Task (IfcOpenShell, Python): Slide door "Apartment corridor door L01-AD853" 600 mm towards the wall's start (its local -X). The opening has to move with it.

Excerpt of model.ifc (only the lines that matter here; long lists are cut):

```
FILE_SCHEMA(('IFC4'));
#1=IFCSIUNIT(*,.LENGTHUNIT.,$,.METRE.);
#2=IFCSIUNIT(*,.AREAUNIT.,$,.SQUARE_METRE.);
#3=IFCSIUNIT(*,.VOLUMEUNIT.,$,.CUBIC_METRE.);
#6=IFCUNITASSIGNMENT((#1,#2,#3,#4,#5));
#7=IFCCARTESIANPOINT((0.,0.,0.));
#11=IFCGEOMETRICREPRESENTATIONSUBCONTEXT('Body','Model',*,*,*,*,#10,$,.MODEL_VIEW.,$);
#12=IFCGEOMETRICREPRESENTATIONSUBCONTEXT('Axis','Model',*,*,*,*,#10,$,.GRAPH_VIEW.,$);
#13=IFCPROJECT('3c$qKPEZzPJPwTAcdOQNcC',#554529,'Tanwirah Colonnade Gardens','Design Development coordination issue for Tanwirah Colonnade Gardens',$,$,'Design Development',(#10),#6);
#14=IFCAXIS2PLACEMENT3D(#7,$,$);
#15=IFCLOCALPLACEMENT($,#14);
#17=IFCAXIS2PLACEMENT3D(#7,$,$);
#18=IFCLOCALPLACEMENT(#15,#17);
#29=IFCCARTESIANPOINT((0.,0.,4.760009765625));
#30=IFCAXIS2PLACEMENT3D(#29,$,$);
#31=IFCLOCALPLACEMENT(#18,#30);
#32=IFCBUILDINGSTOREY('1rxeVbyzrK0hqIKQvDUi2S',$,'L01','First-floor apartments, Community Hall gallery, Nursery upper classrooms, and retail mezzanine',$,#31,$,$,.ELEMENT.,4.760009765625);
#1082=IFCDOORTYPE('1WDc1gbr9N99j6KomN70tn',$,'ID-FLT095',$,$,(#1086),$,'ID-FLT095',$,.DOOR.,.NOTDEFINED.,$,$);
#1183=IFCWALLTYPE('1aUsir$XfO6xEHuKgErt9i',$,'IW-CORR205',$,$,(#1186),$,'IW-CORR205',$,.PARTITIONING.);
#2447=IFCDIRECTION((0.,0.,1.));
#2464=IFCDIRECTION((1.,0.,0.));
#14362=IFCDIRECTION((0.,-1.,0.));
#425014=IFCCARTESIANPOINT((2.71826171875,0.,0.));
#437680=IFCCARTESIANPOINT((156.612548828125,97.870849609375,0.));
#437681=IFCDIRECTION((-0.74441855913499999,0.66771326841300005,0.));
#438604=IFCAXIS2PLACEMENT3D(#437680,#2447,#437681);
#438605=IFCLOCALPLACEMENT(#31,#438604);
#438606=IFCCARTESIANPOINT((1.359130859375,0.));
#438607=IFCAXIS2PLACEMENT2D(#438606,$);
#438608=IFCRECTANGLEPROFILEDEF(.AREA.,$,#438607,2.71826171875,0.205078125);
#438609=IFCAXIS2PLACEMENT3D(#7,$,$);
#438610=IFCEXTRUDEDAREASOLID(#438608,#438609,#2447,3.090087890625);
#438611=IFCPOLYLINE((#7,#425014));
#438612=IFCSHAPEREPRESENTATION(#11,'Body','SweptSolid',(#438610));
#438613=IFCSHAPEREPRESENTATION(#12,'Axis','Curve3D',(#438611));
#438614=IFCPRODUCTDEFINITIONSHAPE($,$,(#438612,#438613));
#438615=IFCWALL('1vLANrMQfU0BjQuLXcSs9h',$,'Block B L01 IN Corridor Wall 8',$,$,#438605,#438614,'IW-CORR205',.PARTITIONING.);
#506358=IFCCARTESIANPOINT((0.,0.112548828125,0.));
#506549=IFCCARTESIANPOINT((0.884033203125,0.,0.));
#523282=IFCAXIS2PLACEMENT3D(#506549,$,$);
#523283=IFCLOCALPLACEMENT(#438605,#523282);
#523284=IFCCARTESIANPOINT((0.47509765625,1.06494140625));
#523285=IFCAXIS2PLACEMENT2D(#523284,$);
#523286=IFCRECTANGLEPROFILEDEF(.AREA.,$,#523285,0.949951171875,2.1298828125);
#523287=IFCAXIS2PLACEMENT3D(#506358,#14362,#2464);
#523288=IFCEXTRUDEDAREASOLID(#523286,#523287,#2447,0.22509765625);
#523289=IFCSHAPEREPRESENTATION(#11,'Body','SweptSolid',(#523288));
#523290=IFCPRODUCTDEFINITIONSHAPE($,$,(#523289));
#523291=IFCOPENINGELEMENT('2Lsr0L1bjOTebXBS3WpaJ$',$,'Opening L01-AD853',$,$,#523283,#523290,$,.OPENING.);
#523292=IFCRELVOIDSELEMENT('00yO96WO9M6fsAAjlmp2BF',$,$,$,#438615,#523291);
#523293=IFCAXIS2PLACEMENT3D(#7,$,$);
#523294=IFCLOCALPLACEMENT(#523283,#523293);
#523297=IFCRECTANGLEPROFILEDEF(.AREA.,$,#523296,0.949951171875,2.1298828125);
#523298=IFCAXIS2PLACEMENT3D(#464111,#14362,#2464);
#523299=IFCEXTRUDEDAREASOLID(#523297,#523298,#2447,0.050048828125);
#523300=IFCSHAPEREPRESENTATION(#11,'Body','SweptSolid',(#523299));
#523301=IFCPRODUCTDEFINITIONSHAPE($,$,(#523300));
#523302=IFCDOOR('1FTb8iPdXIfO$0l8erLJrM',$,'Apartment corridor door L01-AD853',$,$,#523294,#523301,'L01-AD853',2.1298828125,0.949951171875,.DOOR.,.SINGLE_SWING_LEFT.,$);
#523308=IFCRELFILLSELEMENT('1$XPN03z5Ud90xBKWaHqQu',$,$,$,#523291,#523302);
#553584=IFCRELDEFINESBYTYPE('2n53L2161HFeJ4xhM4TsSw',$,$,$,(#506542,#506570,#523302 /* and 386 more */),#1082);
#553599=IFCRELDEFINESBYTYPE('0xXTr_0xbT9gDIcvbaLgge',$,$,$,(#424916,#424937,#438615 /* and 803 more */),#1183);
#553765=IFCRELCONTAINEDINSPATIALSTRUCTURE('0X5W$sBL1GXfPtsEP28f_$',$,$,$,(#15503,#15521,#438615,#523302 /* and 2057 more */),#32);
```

```python
import ifcopenshell
import ifcopenshell.api.geometry
import ifcopenshell.util.placement

model = ifcopenshell.open("model.ifc")

door = model.by_id(523302)
opening = door.FillsVoids[0].RelatingOpeningElement
wall = opening.VoidsElements[0].RelatingBuildingElement

wall_matrix = ifcopenshell.util.placement.get_local_placement(wall.ObjectPlacement)
shift = wall_matrix[:3, 0] * -0.6
before = ifcopenshell.util.placement.get_local_placement(door.ObjectPlacement)[:3, 3].copy()

# The door is placed relative to its opening, so it follows when the opening moves.
matrix = ifcopenshell.util.placement.get_local_placement(opening.ObjectPlacement)
matrix[:3, 3] += shift
ifcopenshell.api.geometry.edit_object_placement(
    model, product=opening, matrix=matrix, is_si=False, should_transform_children=True
)

after = ifcopenshell.util.placement.get_local_placement(door.ObjectPlacement)[:3, 3]
print("door moved by", (after - before).round(3) + 0.0)

model.write("model_updated.ifc")
```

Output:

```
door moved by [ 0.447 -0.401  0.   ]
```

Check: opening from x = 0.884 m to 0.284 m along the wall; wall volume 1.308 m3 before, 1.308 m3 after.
